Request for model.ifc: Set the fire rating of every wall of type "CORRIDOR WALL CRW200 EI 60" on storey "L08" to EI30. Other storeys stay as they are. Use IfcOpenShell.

First a look at what the model holds.

```python
import ifcopenshell
import ifcopenshell.util.element

model = ifcopenshell.open("model.ifc")
print(model.schema)
storey = next(s for s in model.by_type("IfcBuildingStorey") if s.Name == "L08")
walls = [e for e in ifcopenshell.util.element.get_decomposition(storey) if e.is_a("IfcWall")]
seen = {}
for e in walls:
    element_type = ifcopenshell.util.element.get_type(e)
    key = (element_type.Name if element_type != e and element_type else None, ifcopenshell.util.element.get_pset(e, "Pset_WallCommon", "FireRating"))
    seen[key] = seen.get(key, 0) + 1
for (name, value), count in sorted(seen.items(), key=str):
    print(count, "x", name, "|", value)
```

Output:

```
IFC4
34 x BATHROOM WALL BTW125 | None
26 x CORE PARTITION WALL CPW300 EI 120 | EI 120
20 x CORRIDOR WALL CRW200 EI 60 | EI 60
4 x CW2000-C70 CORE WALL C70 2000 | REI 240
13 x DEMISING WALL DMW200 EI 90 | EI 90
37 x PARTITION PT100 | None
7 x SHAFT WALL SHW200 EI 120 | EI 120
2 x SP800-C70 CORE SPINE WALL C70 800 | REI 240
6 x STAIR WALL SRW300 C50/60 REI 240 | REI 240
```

```python
import ifcopenshell
import ifcopenshell.api.pset
import ifcopenshell.util.element

model = ifcopenshell.open("model.ifc")

storey = next(s for s in model.by_type("IfcBuildingStorey") if s.Name == "L08")
walls = [e for e in ifcopenshell.util.element.get_decomposition(storey) if e.is_a("IfcWall")]

count = 0
for e in walls:
    element_type = ifcopenshell.util.element.get_type(e)
    if element_type in (None, e) or element_type.Name != "CORRIDOR WALL CRW200 EI 60":
        continue
    found = ifcopenshell.util.element.get_pset(e, "Pset_WallCommon", should_inherit=False)
    if found:
        pset = model.by_id(found["id"])
        if len(ifcopenshell.util.element.get_elements_by_pset(pset)) > 1:
            pset = ifcopenshell.api.pset.unshare_pset(model, products=[e], pset=pset)[0]
    else:
        pset = ifcopenshell.api.pset.add_pset(model, product=e, name="Pset_WallCommon")
    ifcopenshell.api.pset.edit_pset(model, pset=pset, properties={"FireRating": "EI30"})
    count += 1

print(count, "walls updated")

model.write("model-out.ifc")
```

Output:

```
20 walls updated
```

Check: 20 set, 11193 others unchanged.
